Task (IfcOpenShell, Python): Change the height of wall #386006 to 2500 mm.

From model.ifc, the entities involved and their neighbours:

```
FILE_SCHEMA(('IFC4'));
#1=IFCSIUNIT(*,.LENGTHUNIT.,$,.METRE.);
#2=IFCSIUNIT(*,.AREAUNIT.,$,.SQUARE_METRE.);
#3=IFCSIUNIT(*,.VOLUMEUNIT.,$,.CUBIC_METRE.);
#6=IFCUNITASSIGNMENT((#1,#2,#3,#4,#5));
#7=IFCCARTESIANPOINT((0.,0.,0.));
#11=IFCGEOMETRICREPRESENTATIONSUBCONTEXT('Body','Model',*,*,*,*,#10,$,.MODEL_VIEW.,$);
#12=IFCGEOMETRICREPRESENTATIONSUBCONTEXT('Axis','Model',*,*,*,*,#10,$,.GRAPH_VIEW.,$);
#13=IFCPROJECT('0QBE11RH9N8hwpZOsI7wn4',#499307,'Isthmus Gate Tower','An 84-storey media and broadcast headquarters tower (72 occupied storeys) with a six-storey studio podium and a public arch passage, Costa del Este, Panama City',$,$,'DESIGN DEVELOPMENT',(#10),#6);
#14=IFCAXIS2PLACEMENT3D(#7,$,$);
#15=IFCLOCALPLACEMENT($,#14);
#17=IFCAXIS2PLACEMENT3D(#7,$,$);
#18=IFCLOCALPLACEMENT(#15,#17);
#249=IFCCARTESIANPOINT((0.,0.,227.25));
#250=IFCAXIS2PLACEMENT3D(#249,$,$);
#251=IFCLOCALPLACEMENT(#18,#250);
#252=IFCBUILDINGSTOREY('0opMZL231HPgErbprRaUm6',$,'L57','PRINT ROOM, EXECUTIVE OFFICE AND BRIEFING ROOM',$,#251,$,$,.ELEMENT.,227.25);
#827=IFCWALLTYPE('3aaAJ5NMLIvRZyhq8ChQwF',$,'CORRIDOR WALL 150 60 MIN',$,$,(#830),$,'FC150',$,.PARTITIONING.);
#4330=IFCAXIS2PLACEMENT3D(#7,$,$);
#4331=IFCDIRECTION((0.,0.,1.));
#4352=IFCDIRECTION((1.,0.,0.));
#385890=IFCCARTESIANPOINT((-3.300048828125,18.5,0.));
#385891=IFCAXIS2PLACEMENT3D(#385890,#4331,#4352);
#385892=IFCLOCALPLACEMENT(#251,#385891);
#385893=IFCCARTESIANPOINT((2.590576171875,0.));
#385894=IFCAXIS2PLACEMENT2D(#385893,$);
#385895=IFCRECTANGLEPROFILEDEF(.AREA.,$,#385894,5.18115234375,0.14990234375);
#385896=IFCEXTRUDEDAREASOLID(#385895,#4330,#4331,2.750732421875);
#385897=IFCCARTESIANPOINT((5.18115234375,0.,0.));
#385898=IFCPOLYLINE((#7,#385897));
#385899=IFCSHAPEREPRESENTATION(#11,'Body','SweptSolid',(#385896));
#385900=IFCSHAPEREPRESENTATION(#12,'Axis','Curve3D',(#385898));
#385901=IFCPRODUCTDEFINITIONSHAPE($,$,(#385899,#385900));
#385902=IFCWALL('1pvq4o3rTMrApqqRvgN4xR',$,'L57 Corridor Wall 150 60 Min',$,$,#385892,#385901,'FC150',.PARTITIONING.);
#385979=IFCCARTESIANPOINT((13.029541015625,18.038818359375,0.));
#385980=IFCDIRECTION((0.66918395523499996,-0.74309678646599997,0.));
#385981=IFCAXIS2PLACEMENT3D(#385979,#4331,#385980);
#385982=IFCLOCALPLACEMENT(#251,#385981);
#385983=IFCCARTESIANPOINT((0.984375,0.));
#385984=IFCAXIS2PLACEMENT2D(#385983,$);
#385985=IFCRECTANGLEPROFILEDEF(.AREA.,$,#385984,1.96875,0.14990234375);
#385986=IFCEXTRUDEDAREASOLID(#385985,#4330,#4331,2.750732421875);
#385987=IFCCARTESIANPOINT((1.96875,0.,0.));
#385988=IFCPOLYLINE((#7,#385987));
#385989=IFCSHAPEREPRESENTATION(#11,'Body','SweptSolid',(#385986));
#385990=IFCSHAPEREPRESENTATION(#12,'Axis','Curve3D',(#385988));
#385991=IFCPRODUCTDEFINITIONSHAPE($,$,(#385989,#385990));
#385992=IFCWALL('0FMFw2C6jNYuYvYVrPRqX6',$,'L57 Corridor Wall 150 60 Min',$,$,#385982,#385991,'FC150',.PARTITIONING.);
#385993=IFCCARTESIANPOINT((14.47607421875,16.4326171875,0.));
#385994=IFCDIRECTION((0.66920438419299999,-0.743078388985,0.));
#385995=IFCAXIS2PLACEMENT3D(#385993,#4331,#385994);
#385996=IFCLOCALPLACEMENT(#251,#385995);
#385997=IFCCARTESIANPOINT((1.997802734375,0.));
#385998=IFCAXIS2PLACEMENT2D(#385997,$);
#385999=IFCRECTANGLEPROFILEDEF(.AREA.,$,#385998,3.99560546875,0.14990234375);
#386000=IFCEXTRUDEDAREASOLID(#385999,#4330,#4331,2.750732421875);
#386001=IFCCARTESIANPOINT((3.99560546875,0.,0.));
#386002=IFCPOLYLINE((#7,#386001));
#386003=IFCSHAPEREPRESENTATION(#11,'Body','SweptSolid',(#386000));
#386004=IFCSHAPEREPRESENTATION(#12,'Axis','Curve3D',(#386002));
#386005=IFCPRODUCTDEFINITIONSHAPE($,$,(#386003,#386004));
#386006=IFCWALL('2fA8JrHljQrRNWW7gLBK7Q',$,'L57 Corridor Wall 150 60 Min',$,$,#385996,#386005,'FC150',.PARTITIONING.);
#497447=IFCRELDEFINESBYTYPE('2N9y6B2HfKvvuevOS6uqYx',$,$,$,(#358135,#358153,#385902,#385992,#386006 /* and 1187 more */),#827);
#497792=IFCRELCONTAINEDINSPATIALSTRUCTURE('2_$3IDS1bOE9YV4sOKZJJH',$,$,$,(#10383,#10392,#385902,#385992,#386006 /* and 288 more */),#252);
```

```python
import ifcopenshell
import ifcopenshell.geom
import ifcopenshell.util.representation
import ifcopenshell.util.shape

model = ifcopenshell.open("model.ifc")
settings = ifcopenshell.geom.settings()


def volume(element):
    """Net volume in cubic metres, openings subtracted."""
    shape = ifcopenshell.geom.create_shape(settings, element)
    return ifcopenshell.util.shape.get_volume(shape.geometry)


wall = model.by_id(386006)
before = volume(wall)

body = ifcopenshell.util.representation.get_representation(wall, "Model", "Body")
solid = body.Items[0]
old_height = solid.Depth
solid.Depth = 2.5
after = volume(wall)

print(f"height {old_height:g} -> {solid.Depth:g}, volume {before:.3f} -> {after:.3f} m3")

model.write("model_rev.ifc")
```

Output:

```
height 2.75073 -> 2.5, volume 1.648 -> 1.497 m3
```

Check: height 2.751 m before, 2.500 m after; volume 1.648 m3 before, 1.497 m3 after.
